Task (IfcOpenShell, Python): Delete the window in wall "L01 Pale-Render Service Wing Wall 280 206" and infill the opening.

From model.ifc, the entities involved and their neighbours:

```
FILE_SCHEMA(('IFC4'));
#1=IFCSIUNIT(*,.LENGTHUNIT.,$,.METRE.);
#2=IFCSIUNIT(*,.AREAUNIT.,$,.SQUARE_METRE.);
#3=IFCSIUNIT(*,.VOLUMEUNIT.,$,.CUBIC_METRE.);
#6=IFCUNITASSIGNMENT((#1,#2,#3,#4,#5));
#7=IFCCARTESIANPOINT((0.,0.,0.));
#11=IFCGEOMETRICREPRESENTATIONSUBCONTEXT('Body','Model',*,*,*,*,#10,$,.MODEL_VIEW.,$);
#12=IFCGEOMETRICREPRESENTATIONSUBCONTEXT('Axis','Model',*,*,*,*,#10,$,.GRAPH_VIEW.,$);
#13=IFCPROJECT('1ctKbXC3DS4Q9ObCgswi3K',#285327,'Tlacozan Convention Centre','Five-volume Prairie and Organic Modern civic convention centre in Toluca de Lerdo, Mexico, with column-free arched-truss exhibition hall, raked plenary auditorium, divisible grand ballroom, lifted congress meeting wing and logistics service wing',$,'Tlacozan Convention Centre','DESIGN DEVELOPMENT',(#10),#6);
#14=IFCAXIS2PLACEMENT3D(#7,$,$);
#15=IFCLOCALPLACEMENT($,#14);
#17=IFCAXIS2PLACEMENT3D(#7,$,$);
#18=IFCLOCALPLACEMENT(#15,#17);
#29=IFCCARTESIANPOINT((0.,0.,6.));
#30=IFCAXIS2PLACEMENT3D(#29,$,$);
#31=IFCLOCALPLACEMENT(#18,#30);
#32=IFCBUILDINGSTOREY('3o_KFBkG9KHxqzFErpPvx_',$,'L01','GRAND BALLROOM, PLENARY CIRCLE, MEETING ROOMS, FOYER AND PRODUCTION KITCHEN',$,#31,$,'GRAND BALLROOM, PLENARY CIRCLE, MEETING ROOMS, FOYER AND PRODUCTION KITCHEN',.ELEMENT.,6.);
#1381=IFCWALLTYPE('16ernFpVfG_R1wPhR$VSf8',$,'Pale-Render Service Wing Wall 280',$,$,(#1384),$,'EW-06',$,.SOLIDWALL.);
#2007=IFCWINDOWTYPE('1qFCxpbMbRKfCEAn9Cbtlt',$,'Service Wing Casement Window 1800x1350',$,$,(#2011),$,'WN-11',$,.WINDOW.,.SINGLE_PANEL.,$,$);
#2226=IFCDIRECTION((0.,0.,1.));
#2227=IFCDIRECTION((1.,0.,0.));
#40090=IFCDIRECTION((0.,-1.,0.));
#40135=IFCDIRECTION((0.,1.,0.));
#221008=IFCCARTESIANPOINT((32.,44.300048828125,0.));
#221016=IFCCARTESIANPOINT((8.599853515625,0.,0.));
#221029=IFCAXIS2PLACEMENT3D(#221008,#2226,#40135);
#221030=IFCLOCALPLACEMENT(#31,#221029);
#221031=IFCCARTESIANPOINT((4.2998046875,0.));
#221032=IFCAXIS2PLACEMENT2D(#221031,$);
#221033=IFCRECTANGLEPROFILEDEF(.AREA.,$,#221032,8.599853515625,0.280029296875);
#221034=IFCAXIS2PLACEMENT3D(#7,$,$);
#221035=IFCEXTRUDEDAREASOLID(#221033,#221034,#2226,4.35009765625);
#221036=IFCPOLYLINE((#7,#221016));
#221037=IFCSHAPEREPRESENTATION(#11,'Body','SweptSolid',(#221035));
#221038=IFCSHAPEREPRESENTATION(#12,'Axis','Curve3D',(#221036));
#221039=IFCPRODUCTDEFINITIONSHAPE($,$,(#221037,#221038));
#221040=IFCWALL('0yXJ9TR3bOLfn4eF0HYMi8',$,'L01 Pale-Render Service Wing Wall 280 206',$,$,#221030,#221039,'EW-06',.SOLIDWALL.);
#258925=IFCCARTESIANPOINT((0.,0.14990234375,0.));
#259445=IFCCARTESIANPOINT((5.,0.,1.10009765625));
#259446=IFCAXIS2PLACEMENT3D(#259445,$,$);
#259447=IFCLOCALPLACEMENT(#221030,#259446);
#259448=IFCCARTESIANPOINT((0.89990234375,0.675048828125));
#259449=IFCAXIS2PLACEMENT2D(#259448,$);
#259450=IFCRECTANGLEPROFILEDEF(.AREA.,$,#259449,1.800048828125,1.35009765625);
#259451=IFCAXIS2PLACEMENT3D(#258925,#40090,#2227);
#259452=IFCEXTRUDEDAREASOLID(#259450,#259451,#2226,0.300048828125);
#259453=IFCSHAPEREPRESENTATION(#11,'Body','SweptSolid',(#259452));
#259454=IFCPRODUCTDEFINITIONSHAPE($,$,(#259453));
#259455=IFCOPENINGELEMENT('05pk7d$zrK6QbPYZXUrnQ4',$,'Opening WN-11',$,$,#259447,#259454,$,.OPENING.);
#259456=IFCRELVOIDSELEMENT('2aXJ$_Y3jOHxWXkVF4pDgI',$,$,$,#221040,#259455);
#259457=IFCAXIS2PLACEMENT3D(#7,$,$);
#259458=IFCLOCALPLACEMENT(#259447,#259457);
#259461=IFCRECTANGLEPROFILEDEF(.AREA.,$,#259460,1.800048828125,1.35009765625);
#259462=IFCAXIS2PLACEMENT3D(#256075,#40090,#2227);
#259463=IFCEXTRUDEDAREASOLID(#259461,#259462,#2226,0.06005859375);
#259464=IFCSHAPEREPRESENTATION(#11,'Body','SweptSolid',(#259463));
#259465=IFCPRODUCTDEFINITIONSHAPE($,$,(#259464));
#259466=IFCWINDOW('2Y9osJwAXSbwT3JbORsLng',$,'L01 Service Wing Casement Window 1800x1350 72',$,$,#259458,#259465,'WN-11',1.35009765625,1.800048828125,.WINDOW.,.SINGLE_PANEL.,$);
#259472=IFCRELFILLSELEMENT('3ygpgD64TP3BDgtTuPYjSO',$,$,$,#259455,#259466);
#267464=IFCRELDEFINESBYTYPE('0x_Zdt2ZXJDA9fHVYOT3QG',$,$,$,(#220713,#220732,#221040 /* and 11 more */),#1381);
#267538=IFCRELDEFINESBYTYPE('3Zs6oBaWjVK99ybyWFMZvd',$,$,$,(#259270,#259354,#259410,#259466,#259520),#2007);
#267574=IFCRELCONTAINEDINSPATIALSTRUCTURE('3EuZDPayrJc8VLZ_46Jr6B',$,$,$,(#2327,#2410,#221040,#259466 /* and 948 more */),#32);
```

```python
import ifcopenshell
import ifcopenshell.api.feature
import ifcopenshell.api.root
import ifcopenshell.geom
import ifcopenshell.util.shape

model = ifcopenshell.open("model.ifc")
settings = ifcopenshell.geom.settings()


def volume(element):
    """Net volume in cubic metres, openings subtracted."""
    shape = ifcopenshell.geom.create_shape(settings, element)
    return ifcopenshell.util.shape.get_volume(shape.geometry)


window = model.by_guid("2Y9osJwAXSbwT3JbORsLng")
opening = window.FillsVoids[0].RelatingOpeningElement
wall = opening.VoidsElements[0].RelatingBuildingElement
before = volume(wall)

ifcopenshell.api.root.remove_product(model, product=window)
ifcopenshell.api.feature.remove_feature(model, feature=opening)

after = volume(wall)

print(f"wall volume {before:.3f} -> {after:.3f} m3")

model.write("model_edited.ifc")
```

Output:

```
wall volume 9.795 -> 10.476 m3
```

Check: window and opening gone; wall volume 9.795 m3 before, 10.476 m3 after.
